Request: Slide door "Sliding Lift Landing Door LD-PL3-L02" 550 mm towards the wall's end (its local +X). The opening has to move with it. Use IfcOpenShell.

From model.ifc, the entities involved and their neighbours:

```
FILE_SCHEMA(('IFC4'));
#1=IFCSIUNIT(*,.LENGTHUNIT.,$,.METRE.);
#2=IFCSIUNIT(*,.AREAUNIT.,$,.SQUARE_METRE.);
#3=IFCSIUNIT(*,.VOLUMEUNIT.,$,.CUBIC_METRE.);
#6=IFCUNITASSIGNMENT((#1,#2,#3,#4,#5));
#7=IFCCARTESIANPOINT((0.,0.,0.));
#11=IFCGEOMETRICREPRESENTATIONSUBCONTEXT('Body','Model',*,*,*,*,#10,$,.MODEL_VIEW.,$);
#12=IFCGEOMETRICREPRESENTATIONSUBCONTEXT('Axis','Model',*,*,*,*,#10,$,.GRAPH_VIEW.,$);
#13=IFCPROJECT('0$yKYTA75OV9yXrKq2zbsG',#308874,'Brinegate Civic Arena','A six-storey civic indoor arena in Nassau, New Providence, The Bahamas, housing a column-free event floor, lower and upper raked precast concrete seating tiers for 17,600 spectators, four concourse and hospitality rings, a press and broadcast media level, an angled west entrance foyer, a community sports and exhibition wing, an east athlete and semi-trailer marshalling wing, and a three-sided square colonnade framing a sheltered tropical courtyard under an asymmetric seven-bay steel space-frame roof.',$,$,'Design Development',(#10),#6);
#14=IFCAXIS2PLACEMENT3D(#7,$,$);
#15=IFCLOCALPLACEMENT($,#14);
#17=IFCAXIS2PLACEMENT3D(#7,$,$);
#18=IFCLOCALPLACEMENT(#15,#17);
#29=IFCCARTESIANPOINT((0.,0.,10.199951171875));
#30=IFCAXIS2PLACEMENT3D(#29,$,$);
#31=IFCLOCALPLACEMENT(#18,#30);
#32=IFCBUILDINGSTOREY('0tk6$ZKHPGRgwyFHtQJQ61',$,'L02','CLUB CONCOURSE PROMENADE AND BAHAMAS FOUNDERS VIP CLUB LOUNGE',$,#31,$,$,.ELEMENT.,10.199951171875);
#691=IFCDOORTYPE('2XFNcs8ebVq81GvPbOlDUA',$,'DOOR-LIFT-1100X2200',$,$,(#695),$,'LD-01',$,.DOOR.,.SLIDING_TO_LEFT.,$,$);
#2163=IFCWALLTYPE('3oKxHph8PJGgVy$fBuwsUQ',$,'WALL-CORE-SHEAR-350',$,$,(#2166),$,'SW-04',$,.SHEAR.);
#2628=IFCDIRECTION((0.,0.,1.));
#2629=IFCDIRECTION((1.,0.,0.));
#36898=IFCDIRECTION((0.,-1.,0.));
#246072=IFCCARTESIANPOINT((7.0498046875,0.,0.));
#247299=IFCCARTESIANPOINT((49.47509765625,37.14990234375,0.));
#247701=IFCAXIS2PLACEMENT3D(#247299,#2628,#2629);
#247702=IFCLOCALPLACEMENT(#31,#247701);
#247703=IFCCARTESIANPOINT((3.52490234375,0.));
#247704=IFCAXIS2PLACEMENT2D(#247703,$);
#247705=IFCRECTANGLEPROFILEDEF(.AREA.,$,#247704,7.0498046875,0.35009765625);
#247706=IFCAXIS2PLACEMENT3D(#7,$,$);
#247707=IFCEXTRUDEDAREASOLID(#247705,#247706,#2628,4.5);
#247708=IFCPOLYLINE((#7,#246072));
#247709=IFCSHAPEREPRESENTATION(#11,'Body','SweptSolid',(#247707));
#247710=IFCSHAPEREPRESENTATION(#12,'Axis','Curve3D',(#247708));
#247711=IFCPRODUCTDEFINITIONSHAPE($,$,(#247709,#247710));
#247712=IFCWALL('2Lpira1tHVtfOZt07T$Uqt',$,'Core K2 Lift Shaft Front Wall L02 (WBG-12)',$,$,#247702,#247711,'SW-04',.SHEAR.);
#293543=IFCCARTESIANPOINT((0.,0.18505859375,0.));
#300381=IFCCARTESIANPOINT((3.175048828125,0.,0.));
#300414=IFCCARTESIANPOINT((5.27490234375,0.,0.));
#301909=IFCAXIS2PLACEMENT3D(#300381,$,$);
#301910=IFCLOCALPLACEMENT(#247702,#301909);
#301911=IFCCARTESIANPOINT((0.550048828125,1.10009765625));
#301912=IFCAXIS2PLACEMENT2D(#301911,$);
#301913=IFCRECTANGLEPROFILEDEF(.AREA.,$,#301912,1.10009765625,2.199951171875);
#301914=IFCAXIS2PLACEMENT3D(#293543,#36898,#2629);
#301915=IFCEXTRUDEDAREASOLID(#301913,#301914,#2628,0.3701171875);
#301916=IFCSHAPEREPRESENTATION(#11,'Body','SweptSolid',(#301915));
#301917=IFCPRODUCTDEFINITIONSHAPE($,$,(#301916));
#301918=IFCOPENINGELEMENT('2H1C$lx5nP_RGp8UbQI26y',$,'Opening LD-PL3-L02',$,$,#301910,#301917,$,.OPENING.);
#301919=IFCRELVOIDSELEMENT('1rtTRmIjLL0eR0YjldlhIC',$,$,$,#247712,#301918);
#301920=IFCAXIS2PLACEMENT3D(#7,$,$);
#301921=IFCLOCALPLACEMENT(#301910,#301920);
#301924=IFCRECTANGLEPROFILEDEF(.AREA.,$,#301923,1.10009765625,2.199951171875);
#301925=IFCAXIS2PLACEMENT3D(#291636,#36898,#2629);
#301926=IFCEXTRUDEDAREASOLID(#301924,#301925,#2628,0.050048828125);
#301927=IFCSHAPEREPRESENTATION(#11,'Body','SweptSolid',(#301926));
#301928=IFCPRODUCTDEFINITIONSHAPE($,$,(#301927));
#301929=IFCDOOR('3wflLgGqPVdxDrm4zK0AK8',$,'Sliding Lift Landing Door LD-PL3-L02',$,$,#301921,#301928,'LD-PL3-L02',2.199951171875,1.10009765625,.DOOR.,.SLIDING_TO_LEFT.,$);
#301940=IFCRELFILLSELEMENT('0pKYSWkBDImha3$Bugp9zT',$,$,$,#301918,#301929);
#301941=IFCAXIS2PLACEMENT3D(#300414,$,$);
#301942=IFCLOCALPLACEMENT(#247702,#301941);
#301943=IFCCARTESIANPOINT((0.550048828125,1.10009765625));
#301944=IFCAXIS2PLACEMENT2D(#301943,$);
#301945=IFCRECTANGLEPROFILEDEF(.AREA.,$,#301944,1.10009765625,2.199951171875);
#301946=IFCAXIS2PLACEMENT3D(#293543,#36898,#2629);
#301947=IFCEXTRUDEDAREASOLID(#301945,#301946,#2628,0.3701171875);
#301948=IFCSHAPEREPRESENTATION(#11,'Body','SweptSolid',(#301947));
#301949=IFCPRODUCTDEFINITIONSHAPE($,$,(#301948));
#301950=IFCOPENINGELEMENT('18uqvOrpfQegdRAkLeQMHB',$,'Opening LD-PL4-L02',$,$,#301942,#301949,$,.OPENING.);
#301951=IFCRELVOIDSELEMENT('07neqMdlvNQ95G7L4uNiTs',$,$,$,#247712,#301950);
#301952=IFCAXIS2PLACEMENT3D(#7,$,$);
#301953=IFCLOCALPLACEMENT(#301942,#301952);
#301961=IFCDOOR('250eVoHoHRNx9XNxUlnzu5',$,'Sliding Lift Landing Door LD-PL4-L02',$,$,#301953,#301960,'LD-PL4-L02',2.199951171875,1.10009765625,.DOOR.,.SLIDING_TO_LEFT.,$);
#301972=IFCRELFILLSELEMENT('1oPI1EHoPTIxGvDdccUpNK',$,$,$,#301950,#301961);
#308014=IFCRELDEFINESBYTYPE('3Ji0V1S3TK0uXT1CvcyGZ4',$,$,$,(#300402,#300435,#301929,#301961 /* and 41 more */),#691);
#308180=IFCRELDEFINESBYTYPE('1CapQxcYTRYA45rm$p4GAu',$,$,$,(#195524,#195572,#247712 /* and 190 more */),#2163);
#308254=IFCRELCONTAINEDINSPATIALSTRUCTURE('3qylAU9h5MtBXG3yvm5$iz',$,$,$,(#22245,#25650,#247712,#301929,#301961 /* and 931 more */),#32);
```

```python
import ifcopenshell
import ifcopenshell.api.geometry
import ifcopenshell.util.placement

model = ifcopenshell.open("model.ifc")

door = model.by_id(301929)
opening = door.FillsVoids[0].RelatingOpeningElement
wall = opening.VoidsElements[0].RelatingBuildingElement

wall_matrix = ifcopenshell.util.placement.get_local_placement(wall.ObjectPlacement)
shift = wall_matrix[:3, 0] * 0.55
before = ifcopenshell.util.placement.get_local_placement(door.ObjectPlacement)[:3, 3].copy()

# The door is placed relative to its opening, so it follows when the opening moves.
matrix = ifcopenshell.util.placement.get_local_placement(opening.ObjectPlacement)
matrix[:3, 3] += shift
ifcopenshell.api.geometry.edit_object_placement(
    model, product=opening, matrix=matrix, is_si=False, should_transform_children=True
)

after = ifcopenshell.util.placement.get_local_placement(door.ObjectPlacement)[:3, 3]
print("door moved by", (after - before).round(3) + 0.0)

model.write("model_edited.ifc")
```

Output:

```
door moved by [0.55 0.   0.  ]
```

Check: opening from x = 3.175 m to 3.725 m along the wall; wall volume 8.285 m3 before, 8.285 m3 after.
